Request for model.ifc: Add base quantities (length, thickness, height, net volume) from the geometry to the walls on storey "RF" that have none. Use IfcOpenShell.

First a look at what the model holds.

```python
import ifcopenshell
import ifcopenshell.util.element
import ifcopenshell.util.unit

model = ifcopenshell.open("model.ifc")
print(model.schema)
for unit_type in ("LENGTHUNIT", "AREAUNIT", "VOLUMEUNIT"):
    print(unit_type, ifcopenshell.util.unit.calculate_unit_scale(model, unit_type))
storey = next(s for s in model.by_type("IfcBuildingStorey") if s.Name == "RF")
walls = [e for e in ifcopenshell.util.element.get_decomposition(storey) if e.is_a("IfcWall")]
for e in sorted(walls, key=lambda e: e.id()):
    print(e.id(), e.is_a(), e.Name, list(ifcopenshell.util.element.get_psets(e, qtos_only=True)), sep=" | ")
```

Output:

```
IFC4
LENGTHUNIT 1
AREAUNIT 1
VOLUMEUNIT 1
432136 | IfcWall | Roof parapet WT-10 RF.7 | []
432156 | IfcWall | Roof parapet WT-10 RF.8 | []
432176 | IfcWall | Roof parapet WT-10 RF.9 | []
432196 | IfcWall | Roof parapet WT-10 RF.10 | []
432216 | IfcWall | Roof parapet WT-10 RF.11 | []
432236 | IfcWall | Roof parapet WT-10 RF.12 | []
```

```python
import ifcopenshell
import ifcopenshell.api.pset
import ifcopenshell.geom
import ifcopenshell.util.element
import ifcopenshell.util.shape
import ifcopenshell.util.unit

model = ifcopenshell.open("model.ifc")
unit_scale = ifcopenshell.util.unit.calculate_unit_scale(model)
volume_scale = ifcopenshell.util.unit.calculate_unit_scale(model, "VOLUMEUNIT")
settings = ifcopenshell.geom.settings()

storey = next(s for s in model.by_type("IfcBuildingStorey") if s.Name == "RF")
walls = [e for e in ifcopenshell.util.element.get_decomposition(storey) if e.is_a("IfcWall")]

for e in sorted(walls, key=lambda e: e.id()):
    if ifcopenshell.util.element.get_psets(e, qtos_only=True, should_inherit=False):
        continue
    # Geometry comes back in metres, in the element's own axes.
    shape = ifcopenshell.geom.create_shape(settings, e)
    values = {
        "Length": ifcopenshell.util.shape.get_x(shape.geometry) / unit_scale,
        "Width": ifcopenshell.util.shape.get_y(shape.geometry) / unit_scale,
        "Height": ifcopenshell.util.shape.get_z(shape.geometry) / unit_scale,
        "NetVolume": ifcopenshell.util.shape.get_volume(shape.geometry) / volume_scale,
    }
    qto = ifcopenshell.api.pset.add_qto(model, product=e, name="Qto_WallBaseQuantities")
    ifcopenshell.api.pset.edit_qto(model, qto=qto, properties=values)
    print(e.id(), {k: round(v, 3) for k, v in values.items()})

model.write("model_updated.ifc")
```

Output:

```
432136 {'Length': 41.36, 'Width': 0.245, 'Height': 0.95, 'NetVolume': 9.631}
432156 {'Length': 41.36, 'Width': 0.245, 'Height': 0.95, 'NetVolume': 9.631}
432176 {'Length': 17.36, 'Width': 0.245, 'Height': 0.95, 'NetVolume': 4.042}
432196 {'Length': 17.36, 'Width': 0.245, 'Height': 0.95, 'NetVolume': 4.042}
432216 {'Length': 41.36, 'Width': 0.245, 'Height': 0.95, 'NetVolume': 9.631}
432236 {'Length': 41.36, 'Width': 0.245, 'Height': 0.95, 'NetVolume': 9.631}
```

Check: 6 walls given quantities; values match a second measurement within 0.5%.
